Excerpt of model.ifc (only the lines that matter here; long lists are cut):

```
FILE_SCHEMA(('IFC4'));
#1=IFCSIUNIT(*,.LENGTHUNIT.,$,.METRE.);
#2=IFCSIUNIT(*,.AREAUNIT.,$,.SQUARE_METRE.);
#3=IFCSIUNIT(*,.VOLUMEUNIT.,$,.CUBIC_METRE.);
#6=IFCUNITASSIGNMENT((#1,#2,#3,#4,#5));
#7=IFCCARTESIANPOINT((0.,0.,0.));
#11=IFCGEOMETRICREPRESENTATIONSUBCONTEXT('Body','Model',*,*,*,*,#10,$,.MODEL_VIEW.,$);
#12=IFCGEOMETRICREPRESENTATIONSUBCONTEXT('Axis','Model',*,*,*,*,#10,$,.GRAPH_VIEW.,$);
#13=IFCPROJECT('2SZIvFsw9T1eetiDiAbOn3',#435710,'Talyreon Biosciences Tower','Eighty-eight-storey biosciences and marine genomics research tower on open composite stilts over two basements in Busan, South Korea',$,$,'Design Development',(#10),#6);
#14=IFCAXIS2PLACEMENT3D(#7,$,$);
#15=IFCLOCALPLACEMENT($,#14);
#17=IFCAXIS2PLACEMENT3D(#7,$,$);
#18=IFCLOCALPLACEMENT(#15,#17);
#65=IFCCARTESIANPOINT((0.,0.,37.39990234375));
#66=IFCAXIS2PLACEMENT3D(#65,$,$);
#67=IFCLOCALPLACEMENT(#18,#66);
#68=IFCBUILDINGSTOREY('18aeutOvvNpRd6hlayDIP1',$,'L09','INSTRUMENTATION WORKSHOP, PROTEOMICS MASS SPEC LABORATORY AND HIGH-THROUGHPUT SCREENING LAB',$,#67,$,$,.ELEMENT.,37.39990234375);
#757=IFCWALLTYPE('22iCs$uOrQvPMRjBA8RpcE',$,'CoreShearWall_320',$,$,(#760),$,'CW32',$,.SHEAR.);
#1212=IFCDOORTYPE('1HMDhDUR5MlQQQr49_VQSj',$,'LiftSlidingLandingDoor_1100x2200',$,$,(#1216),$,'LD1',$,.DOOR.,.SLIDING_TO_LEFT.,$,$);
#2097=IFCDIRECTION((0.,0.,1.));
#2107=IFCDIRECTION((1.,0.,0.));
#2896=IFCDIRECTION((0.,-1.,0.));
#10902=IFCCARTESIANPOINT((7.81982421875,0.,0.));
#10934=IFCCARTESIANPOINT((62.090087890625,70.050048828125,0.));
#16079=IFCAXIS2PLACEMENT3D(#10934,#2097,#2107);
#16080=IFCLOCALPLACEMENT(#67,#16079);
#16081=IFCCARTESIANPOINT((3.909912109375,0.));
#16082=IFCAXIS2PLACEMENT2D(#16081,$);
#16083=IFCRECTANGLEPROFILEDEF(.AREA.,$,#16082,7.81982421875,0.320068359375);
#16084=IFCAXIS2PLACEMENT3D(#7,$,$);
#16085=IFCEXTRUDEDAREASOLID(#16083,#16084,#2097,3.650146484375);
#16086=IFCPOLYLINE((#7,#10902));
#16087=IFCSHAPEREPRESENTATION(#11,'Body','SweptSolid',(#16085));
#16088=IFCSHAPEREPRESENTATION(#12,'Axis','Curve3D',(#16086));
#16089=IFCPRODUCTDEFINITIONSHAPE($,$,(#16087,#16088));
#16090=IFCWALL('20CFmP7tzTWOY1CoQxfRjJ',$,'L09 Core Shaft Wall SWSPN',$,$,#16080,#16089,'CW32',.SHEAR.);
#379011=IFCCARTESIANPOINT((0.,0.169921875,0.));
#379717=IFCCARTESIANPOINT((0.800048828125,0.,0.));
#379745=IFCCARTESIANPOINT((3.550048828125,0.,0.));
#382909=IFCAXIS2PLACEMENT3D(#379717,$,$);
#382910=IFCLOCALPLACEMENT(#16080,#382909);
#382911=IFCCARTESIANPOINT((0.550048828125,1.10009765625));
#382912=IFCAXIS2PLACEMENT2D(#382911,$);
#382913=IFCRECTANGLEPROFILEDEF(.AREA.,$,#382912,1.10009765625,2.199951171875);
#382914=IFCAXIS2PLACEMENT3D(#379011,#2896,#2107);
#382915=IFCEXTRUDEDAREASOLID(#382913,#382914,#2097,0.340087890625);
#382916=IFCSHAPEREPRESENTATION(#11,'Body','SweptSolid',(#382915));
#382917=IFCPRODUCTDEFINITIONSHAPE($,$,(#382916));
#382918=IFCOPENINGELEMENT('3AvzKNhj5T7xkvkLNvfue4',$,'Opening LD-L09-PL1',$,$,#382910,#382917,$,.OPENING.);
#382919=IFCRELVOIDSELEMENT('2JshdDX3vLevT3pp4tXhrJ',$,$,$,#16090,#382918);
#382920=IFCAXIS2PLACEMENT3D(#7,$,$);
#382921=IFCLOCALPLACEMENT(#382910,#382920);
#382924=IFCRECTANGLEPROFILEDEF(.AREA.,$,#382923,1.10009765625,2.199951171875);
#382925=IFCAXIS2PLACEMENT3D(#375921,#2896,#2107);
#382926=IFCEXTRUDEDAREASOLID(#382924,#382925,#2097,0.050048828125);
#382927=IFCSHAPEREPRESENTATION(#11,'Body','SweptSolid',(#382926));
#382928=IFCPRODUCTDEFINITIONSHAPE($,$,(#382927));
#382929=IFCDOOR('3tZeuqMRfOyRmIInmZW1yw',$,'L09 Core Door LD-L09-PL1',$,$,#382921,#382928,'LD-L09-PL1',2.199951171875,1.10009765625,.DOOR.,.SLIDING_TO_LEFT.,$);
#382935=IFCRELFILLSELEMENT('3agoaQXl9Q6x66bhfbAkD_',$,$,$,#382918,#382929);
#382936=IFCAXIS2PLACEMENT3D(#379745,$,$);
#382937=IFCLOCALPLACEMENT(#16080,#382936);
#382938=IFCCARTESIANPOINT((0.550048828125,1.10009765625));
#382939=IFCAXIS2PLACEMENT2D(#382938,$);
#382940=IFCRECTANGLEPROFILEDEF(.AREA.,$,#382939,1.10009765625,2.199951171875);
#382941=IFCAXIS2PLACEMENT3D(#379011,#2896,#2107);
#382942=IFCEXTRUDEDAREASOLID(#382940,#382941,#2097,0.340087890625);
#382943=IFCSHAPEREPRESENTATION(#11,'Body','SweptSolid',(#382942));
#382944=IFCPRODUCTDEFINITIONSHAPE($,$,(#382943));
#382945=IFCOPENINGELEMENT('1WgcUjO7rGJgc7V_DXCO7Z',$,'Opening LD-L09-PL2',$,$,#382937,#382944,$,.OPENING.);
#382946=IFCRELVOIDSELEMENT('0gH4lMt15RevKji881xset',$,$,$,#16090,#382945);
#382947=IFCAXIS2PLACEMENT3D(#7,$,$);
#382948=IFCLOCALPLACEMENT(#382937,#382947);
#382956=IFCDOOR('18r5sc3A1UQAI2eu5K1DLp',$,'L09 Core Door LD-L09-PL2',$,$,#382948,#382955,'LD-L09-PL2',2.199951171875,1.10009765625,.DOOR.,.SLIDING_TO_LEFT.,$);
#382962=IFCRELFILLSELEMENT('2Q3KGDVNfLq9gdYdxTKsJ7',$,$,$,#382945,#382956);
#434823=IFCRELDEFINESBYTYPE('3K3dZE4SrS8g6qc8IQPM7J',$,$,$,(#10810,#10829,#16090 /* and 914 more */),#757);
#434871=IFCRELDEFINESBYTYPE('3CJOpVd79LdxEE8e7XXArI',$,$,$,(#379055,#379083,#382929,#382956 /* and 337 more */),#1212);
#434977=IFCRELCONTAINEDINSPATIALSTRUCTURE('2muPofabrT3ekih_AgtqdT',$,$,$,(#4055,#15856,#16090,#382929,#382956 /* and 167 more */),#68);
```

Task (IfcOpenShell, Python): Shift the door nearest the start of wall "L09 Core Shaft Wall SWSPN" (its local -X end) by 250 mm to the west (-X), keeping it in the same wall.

```python
import ifcopenshell
import ifcopenshell.api.geometry
import ifcopenshell.util.placement

model = ifcopenshell.open("model.ifc")

door = model.by_guid("3tZeuqMRfOyRmIInmZW1yw")
opening = door.FillsVoids[0].RelatingOpeningElement
wall = opening.VoidsElements[0].RelatingBuildingElement

wall_matrix = ifcopenshell.util.placement.get_local_placement(wall.ObjectPlacement)
shift = wall_matrix[:3, 0] * -0.25
before = ifcopenshell.util.placement.get_local_placement(door.ObjectPlacement)[:3, 3].copy()

# The door is placed relative to its opening, so it follows when the opening moves.
matrix = ifcopenshell.util.placement.get_local_placement(opening.ObjectPlacement)
matrix[:3, 3] += shift
ifcopenshell.api.geometry.edit_object_placement(
    model, product=opening, matrix=matrix, is_si=False, should_transform_children=True
)

after = ifcopenshell.util.placement.get_local_placement(door.ObjectPlacement)[:3, 3]
print("door moved by", (after - before).round(3) + 0.0)

model.write("model_edited.ifc")
```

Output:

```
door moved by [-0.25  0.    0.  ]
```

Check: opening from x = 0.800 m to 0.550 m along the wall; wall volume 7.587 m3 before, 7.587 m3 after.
